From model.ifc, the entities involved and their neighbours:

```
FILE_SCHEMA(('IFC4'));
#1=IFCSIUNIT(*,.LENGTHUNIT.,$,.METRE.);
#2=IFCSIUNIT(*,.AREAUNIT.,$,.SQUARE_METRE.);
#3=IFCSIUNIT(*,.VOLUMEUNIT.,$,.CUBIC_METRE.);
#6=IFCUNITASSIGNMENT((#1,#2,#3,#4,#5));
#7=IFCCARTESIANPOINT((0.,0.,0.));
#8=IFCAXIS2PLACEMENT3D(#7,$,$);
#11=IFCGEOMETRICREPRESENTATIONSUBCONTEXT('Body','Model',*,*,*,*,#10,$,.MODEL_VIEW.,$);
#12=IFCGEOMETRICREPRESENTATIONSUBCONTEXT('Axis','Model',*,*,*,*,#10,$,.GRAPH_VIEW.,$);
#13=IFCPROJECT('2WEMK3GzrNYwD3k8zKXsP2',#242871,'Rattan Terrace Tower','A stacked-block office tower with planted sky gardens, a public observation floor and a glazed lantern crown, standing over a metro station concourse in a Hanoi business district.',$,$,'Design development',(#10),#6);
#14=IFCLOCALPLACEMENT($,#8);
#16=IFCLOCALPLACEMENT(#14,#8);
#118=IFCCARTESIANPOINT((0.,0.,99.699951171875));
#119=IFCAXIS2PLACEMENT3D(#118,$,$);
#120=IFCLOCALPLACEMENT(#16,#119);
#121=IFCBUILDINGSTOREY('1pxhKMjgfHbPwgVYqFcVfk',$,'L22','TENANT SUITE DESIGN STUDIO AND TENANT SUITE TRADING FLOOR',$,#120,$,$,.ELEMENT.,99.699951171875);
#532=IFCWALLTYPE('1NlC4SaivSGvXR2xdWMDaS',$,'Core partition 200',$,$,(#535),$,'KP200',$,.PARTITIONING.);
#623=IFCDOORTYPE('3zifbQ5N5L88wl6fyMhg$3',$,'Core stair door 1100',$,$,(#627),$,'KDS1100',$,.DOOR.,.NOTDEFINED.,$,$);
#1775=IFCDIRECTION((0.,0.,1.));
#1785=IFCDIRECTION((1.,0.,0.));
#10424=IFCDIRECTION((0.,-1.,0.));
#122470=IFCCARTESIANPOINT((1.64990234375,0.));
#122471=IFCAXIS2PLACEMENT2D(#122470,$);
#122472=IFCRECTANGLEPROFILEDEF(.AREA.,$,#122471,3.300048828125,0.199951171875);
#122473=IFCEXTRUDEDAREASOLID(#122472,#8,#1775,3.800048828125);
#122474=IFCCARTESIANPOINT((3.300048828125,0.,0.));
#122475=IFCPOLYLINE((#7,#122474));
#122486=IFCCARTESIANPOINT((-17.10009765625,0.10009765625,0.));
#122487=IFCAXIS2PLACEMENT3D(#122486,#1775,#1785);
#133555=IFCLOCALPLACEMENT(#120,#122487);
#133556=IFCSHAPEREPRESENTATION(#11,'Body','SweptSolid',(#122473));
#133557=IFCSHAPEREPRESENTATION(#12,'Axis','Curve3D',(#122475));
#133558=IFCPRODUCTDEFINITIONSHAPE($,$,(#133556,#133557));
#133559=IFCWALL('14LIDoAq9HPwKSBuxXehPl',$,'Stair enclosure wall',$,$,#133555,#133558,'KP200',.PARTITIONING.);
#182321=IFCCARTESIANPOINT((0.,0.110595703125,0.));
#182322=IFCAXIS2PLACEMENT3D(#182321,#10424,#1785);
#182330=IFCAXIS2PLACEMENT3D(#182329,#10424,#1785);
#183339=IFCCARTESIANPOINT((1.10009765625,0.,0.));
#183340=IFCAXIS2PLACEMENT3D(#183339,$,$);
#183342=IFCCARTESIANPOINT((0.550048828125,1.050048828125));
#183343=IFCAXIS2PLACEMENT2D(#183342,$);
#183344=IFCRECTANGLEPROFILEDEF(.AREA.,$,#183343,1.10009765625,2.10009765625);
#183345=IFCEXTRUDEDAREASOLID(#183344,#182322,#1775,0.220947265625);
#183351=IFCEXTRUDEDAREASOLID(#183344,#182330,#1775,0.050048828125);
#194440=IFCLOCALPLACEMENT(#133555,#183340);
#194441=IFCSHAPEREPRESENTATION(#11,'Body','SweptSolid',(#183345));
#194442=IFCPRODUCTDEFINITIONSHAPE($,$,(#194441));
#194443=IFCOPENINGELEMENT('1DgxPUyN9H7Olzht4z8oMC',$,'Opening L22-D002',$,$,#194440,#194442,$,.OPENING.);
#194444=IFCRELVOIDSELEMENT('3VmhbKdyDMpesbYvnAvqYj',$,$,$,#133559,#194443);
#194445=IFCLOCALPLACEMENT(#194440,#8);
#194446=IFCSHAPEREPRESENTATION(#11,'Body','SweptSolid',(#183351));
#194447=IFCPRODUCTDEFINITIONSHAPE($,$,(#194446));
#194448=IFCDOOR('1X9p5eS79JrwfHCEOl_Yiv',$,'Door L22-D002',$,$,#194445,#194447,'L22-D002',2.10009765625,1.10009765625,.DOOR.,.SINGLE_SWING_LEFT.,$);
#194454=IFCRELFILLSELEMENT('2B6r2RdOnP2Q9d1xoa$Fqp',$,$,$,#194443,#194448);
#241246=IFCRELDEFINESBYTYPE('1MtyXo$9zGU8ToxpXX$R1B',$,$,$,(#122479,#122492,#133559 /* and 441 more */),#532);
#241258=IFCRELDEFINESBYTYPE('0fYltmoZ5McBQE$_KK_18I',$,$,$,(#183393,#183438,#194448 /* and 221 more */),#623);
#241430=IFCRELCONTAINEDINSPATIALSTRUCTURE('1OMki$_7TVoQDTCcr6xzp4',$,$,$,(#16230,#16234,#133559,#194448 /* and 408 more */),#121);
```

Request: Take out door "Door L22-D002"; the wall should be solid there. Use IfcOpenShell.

```python
import ifcopenshell
import ifcopenshell.api.feature
import ifcopenshell.api.root
import ifcopenshell.geom
import ifcopenshell.util.shape

model = ifcopenshell.open("model.ifc")
settings = ifcopenshell.geom.settings()


def volume(element):
    """Net volume in cubic metres, openings subtracted."""
    shape = ifcopenshell.geom.create_shape(settings, element)
    return ifcopenshell.util.shape.get_volume(shape.geometry)


door = model.by_guid("1X9p5eS79JrwfHCEOl_Yiv")
opening = door.FillsVoids[0].RelatingOpeningElement
wall = opening.VoidsElements[0].RelatingBuildingElement
before = volume(wall)

ifcopenshell.api.root.remove_product(model, product=door)
ifcopenshell.api.feature.remove_feature(model, feature=opening)

after = volume(wall)

print(f"wall volume {before:.3f} -> {after:.3f} m3")

model.write("model_rev.ifc")
```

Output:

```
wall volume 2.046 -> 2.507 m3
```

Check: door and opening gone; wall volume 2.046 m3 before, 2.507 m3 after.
